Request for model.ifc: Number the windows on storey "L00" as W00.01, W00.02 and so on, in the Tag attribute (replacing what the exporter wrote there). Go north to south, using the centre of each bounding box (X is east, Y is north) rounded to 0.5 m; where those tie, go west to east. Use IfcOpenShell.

First a look at what the model holds.

```python
import ifcopenshell
import ifcopenshell.util.element
import ifcopenshell.util.placement

model = ifcopenshell.open("model.ifc")
print(model.schema)
storey = next(s for s in model.by_type("IfcBuildingStorey") if s.Name == "L00")
windows = [e for e in ifcopenshell.util.element.get_decomposition(storey) if e.is_a("IfcWindow")]
for e in sorted(windows, key=lambda e: e.id()):
    origin = ifcopenshell.util.placement.get_local_placement(e.ObjectPlacement)[:3, 3]
    print(e.id(), e.Tag, e.Name, origin.round(2) + 0.0, sep=" | ")
```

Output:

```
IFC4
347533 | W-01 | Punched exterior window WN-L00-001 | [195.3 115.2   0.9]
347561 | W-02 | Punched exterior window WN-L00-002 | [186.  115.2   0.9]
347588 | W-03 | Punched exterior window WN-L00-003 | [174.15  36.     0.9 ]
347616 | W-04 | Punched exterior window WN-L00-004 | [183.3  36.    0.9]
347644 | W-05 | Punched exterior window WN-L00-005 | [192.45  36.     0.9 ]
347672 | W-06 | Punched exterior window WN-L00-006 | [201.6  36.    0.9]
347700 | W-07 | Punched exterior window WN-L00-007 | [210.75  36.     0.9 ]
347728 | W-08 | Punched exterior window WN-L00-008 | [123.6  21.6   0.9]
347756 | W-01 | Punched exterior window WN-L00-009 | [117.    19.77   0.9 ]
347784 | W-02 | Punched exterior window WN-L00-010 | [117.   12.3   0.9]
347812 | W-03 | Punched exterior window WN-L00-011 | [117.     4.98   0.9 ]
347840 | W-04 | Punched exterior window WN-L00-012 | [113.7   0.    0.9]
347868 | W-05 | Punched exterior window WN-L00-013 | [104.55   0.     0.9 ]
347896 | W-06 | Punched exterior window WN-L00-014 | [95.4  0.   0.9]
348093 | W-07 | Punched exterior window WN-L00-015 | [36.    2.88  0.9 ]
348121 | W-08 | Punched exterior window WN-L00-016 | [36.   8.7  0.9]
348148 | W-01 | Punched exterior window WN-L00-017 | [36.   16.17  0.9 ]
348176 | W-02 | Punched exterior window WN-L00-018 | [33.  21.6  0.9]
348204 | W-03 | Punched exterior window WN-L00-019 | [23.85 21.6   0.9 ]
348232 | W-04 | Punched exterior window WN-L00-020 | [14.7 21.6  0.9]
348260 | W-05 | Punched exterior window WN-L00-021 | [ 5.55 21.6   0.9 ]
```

```python
import ifcopenshell
import ifcopenshell.geom
import ifcopenshell.util.element
import ifcopenshell.util.shape

model = ifcopenshell.open("model.ifc")
settings = ifcopenshell.geom.settings()
settings.set("use-world-coords", True)


def centre(element):
    shape = ifcopenshell.geom.create_shape(settings, element)
    return ifcopenshell.util.shape.get_bbox_centroid(shape.geometry)


storey = next(s for s in model.by_type("IfcBuildingStorey") if s.Name == "L00")
windows = [e for e in ifcopenshell.util.element.get_decomposition(storey) if e.is_a("IfcWindow")]

# Insertion points can sit at a corner or the storey origin, so sort by the geometry (in metres).
centres = {e: centre(e) for e in windows}
windows.sort(key=lambda e: (-round(centres[e][1] / 0.5), centres[e][0]))

for i, e in enumerate(windows, start=1):
    number = f"W00.{i:02d}"
    e.Tag = number
    print(e.id(), number)

model.write("model_updated.ifc")
```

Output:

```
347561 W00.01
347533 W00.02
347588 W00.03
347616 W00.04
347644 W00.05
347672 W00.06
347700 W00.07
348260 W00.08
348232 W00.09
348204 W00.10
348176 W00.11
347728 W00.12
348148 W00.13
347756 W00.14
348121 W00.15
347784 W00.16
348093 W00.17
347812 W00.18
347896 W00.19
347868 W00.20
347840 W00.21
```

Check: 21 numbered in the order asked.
